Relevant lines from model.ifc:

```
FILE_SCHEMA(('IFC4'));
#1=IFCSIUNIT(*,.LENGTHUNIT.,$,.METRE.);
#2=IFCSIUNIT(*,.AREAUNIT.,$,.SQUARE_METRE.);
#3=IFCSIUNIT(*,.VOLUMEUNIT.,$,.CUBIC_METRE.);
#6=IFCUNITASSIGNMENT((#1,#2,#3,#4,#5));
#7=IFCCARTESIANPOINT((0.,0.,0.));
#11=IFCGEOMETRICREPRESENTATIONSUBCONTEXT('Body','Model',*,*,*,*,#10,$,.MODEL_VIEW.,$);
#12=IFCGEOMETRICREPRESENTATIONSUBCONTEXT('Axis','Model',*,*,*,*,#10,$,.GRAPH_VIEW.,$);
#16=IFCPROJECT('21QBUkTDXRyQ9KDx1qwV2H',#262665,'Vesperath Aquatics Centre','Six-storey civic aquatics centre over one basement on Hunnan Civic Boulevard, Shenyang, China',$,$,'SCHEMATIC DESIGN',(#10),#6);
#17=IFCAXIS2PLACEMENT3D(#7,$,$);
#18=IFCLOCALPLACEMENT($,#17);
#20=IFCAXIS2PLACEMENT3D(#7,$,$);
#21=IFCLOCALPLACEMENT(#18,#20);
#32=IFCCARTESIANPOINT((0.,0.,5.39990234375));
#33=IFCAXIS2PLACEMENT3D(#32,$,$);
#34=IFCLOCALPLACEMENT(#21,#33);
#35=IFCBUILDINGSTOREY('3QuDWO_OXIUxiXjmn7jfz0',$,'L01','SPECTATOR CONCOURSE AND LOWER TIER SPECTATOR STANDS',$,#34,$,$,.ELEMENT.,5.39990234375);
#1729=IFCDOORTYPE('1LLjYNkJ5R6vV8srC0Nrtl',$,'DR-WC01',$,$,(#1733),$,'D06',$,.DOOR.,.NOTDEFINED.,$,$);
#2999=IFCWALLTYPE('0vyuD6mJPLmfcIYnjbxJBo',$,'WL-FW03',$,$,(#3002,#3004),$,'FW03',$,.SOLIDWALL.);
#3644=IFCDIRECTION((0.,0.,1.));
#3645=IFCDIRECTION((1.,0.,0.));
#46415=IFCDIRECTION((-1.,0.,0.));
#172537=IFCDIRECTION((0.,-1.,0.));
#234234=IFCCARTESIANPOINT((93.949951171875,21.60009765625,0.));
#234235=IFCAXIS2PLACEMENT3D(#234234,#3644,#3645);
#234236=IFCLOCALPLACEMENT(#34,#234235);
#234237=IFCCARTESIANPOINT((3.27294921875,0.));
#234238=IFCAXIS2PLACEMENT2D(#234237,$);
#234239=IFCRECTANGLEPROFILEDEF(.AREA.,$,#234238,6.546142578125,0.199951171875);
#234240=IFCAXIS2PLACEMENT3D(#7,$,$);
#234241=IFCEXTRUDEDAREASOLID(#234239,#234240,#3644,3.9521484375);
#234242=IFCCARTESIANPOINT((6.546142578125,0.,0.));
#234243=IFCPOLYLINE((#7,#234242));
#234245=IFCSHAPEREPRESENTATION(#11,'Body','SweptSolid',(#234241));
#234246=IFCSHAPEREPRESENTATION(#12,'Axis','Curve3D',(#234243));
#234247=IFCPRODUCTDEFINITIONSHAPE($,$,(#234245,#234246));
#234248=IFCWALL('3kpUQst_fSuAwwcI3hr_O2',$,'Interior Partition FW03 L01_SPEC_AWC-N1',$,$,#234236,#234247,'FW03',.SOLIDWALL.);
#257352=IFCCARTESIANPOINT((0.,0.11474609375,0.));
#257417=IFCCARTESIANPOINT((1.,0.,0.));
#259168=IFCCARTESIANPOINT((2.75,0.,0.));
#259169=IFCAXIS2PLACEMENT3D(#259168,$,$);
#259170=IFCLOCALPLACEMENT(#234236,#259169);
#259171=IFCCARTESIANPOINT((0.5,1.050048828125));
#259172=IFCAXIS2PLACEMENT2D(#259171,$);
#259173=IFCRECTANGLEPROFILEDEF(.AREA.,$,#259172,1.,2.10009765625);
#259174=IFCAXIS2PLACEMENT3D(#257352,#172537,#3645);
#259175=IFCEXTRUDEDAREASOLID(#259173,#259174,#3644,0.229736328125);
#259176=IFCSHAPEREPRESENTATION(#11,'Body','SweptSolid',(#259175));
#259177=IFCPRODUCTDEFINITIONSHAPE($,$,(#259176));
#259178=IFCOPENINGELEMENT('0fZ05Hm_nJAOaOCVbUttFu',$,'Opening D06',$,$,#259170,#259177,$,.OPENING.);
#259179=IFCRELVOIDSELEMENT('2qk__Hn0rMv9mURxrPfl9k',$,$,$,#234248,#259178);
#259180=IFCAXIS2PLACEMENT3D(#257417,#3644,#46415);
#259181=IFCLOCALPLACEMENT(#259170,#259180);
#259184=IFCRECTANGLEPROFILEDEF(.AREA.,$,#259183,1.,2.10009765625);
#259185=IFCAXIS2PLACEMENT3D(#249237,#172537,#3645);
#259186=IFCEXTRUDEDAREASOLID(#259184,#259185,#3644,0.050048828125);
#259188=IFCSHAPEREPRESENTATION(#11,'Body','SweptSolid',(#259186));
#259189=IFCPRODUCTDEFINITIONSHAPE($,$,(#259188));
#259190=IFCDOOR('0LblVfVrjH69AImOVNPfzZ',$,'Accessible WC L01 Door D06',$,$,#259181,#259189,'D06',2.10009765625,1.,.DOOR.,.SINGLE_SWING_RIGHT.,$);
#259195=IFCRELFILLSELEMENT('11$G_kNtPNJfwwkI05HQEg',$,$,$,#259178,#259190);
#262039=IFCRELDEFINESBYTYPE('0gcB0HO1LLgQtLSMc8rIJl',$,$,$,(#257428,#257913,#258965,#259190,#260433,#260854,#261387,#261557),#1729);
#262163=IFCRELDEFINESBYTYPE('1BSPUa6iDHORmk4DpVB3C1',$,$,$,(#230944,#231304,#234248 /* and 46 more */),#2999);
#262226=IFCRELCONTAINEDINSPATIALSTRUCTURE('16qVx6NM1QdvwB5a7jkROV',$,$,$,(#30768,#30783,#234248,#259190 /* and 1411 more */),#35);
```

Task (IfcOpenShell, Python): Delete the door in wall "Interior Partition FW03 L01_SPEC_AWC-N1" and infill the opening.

```python
import ifcopenshell
import ifcopenshell.api.feature
import ifcopenshell.api.root
import ifcopenshell.geom
import ifcopenshell.util.shape

model = ifcopenshell.open("model.ifc")
settings = ifcopenshell.geom.settings()


def volume(element):
    """Net volume in cubic metres, openings subtracted."""
    shape = ifcopenshell.geom.create_shape(settings, element)
    return ifcopenshell.util.shape.get_volume(shape.geometry)


door = model.by_guid("0LblVfVrjH69AImOVNPfzZ")
opening = door.FillsVoids[0].RelatingOpeningElement
wall = opening.VoidsElements[0].RelatingBuildingElement
before = volume(wall)

ifcopenshell.api.root.remove_product(model, product=door)
ifcopenshell.api.feature.remove_feature(model, feature=opening)

after = volume(wall)

print(f"wall volume {before:.3f} -> {after:.3f} m3")

model.write("model_rev.ifc")
```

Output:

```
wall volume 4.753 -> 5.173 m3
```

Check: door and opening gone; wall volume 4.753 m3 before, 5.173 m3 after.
